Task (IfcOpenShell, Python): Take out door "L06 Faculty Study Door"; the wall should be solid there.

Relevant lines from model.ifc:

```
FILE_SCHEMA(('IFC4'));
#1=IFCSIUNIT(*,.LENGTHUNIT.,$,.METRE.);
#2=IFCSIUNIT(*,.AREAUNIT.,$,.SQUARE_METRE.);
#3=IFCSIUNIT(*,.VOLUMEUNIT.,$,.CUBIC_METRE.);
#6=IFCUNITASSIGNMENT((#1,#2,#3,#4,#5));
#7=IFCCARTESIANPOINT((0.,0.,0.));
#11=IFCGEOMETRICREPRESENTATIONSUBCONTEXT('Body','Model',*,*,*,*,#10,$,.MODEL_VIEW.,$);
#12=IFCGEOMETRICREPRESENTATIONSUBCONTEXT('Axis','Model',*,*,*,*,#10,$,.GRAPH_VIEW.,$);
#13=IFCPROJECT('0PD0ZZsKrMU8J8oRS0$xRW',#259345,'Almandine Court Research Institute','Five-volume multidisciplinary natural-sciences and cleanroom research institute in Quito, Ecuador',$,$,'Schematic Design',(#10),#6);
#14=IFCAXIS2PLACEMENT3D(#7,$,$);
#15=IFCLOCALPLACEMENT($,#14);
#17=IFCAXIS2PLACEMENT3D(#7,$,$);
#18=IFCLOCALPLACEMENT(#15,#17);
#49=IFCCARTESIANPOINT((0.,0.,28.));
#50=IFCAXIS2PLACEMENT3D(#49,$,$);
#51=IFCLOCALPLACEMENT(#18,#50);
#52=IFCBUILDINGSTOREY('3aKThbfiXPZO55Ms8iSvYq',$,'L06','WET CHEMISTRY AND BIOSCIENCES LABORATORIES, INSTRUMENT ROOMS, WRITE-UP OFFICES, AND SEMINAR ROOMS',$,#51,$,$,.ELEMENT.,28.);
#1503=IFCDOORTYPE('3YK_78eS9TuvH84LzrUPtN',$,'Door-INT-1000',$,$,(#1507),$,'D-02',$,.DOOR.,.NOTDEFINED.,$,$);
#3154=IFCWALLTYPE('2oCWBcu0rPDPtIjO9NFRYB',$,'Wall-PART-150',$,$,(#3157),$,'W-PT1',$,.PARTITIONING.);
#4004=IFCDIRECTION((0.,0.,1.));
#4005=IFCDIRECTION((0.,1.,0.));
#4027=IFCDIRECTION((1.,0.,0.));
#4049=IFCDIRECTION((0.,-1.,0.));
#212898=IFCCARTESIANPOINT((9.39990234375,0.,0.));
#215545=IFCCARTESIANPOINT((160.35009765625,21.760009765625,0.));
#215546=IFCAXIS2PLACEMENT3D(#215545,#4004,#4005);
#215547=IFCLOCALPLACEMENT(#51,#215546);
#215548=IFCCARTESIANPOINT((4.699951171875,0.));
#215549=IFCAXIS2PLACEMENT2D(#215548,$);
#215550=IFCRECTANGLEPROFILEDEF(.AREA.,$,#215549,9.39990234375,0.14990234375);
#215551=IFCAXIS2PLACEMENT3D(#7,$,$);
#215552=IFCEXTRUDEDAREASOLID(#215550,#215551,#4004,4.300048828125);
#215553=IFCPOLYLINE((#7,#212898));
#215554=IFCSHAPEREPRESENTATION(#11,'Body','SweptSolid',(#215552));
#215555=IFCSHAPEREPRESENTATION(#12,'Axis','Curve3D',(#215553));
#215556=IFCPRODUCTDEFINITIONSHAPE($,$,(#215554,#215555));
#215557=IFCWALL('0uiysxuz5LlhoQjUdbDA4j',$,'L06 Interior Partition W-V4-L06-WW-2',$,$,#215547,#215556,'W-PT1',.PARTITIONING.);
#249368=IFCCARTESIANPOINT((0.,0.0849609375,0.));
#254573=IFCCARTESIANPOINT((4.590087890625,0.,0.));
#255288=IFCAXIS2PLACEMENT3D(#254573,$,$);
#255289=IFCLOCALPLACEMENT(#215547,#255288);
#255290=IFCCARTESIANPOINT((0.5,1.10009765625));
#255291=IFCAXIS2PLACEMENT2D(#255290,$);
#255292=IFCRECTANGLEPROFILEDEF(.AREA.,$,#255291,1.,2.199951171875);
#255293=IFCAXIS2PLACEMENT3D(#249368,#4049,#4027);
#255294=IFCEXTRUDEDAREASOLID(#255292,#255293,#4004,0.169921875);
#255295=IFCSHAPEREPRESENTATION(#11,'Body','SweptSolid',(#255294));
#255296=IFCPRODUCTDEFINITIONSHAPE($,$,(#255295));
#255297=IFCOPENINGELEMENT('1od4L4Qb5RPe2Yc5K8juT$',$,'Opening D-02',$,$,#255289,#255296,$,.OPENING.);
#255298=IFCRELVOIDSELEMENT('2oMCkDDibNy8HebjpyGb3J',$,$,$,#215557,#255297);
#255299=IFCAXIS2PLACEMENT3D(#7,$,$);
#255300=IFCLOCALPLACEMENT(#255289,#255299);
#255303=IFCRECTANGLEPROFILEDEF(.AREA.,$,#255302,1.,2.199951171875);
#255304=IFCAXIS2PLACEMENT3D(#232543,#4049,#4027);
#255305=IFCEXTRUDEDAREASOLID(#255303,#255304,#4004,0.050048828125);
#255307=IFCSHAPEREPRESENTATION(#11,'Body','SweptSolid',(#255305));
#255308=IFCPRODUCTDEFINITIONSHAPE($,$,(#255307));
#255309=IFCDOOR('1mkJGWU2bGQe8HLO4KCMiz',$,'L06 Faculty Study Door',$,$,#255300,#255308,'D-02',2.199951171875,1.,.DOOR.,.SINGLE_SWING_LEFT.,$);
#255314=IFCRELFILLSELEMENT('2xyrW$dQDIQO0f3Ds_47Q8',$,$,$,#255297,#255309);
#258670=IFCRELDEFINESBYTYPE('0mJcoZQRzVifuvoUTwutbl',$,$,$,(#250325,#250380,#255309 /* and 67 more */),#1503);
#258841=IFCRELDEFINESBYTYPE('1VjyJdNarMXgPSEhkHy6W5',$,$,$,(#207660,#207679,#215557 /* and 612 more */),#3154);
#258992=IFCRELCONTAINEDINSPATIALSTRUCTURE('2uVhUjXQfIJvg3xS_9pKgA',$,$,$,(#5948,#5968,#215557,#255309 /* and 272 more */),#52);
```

```python
import ifcopenshell
import ifcopenshell.api.feature
import ifcopenshell.api.root
import ifcopenshell.geom
import ifcopenshell.util.shape

model = ifcopenshell.open("model.ifc")
settings = ifcopenshell.geom.settings()


def volume(element):
    """Net volume in cubic metres, openings subtracted."""
    shape = ifcopenshell.geom.create_shape(settings, element)
    return ifcopenshell.util.shape.get_volume(shape.geometry)


door = model.by_guid("1mkJGWU2bGQe8HLO4KCMiz")
opening = door.FillsVoids[0].RelatingOpeningElement
wall = opening.VoidsElements[0].RelatingBuildingElement
before = volume(wall)

ifcopenshell.api.root.remove_product(model, product=door)
ifcopenshell.api.feature.remove_feature(model, feature=opening)

after = volume(wall)

print(f"wall volume {before:.3f} -> {after:.3f} m3")

model.write("model_v2.ifc")
```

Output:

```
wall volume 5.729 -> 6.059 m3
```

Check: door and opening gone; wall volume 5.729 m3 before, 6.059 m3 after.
